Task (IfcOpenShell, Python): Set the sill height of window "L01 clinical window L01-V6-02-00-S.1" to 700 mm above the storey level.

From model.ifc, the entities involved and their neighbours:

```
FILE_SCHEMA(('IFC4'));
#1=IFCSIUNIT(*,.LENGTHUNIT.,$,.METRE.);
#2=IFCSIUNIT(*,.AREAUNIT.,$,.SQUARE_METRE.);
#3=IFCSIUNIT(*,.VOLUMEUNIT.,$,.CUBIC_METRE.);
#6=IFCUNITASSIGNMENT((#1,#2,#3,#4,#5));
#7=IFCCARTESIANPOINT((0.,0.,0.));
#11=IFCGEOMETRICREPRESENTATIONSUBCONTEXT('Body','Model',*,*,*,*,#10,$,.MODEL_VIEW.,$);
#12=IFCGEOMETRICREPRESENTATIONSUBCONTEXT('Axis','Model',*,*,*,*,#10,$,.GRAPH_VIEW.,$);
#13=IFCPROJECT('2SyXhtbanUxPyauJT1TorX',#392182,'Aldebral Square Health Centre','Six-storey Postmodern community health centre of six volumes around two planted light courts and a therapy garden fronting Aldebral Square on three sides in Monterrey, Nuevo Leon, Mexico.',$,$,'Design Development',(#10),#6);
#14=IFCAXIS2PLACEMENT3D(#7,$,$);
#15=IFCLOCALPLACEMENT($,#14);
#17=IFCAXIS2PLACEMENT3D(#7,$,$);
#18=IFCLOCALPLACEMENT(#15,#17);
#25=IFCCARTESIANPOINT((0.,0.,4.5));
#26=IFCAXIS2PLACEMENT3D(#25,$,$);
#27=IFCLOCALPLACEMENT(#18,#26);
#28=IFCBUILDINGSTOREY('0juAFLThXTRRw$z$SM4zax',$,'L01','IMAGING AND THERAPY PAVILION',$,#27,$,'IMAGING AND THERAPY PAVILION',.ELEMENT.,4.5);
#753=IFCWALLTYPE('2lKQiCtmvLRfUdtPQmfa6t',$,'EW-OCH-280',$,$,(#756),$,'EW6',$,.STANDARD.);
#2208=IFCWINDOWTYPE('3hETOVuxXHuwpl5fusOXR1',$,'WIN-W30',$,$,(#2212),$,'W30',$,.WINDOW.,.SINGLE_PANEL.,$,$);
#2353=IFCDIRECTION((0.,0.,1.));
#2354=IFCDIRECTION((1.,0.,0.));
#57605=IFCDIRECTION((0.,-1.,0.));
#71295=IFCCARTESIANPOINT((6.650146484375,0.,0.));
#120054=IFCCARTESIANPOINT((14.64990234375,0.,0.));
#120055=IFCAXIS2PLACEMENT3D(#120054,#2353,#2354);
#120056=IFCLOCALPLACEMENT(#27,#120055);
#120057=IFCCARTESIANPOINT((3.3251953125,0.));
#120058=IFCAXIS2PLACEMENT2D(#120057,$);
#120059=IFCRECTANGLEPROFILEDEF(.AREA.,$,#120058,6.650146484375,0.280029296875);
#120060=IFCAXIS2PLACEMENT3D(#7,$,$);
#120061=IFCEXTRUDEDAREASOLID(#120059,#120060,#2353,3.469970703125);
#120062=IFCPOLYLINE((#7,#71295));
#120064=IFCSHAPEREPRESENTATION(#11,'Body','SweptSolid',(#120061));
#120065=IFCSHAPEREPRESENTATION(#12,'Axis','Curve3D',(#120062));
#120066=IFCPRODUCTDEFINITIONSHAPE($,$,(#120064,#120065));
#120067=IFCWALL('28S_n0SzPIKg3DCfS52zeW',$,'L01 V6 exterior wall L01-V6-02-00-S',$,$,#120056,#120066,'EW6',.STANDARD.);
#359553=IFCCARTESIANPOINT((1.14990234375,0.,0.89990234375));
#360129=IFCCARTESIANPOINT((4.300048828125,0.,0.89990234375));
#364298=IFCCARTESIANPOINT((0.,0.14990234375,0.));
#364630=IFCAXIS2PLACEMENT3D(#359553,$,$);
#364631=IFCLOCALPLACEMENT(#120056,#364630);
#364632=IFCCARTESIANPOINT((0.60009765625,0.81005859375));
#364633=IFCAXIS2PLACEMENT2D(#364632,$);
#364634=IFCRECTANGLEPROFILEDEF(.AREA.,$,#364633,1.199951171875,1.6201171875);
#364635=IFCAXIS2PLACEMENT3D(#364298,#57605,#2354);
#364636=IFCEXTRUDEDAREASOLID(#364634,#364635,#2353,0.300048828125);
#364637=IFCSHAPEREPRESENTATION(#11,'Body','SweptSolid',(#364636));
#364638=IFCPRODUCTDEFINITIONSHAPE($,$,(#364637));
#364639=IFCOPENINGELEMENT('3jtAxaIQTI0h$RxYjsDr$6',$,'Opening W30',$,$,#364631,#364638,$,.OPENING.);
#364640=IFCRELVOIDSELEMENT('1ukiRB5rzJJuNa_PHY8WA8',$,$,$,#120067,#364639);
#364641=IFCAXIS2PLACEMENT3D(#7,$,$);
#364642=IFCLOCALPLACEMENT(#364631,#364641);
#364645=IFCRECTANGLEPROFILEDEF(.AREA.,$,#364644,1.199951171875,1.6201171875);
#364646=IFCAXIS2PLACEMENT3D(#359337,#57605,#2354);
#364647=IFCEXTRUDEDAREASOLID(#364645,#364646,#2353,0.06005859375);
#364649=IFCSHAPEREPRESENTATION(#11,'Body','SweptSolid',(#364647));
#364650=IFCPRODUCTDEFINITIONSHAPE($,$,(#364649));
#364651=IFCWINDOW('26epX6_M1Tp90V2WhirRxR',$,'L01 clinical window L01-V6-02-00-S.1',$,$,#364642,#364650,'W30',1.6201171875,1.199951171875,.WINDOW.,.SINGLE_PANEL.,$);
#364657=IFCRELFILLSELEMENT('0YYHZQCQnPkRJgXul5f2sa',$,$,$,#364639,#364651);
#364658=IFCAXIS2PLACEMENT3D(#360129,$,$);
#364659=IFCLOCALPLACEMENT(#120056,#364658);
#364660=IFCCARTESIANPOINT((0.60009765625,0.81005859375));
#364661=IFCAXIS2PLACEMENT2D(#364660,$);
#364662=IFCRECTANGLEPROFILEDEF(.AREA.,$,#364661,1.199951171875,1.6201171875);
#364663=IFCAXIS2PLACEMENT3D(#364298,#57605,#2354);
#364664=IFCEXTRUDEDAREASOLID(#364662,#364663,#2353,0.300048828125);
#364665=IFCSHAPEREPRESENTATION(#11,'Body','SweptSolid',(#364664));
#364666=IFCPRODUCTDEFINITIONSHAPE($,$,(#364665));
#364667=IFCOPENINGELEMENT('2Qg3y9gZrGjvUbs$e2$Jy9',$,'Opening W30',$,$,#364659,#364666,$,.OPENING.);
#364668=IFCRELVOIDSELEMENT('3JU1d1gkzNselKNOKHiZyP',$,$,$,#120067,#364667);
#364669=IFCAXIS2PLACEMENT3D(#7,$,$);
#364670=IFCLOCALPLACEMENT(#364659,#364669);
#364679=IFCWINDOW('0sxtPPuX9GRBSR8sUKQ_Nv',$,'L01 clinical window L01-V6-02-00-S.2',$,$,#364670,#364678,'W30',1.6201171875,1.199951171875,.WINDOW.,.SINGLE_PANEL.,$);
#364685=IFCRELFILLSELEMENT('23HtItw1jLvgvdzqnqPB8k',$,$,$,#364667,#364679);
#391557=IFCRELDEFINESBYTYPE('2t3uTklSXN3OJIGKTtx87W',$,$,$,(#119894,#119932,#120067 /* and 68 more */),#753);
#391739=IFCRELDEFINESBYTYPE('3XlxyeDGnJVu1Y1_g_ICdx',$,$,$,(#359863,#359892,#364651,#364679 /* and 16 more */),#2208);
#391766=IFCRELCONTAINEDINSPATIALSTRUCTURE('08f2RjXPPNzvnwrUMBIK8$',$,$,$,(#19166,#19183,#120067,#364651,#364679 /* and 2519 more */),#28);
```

```python
import numpy as np
import ifcopenshell
import ifcopenshell.api.geometry
import ifcopenshell.geom
import ifcopenshell.util.element
import ifcopenshell.util.placement
import ifcopenshell.util.shape
import ifcopenshell.util.unit

model = ifcopenshell.open("model.ifc")
unit_scale = ifcopenshell.util.unit.calculate_unit_scale(model)

window = model.by_id(364651)
opening = window.FillsVoids[0].RelatingOpeningElement
storey = ifcopenshell.util.element.get_container(window, ifc_class="IfcBuildingStorey")
level = ifcopenshell.util.placement.get_local_placement(storey.ObjectPlacement)[2, 3]

# The opening's origin need not be at the sill, so measure its lowest point.
shape = ifcopenshell.geom.create_shape(ifcopenshell.geom.settings(), opening)
bottom = ifcopenshell.util.shape.get_shape_bottom_elevation(shape, shape.geometry) / unit_scale
dz = level + 0.7 / unit_scale - bottom

shift = np.array([0.0, 0.0, dz])
# The window is placed relative to its opening, so it follows when the opening moves.
matrix = ifcopenshell.util.placement.get_local_placement(opening.ObjectPlacement)
matrix[:3, 3] += shift
ifcopenshell.api.geometry.edit_object_placement(
    model, product=opening, matrix=matrix, is_si=False, should_transform_children=True
)

print(f"moved by {dz * unit_scale:+.3f} m")

model.write("model_rev.ifc")
```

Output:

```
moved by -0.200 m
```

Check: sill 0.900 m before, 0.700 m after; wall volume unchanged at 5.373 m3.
